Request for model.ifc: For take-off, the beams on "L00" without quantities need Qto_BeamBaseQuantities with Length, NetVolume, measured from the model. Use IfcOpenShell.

First a look at what the model holds.

```python
import ifcopenshell
import ifcopenshell.util.element
import ifcopenshell.util.unit

model = ifcopenshell.open("model.ifc")
print(model.schema)
for unit_type in ("LENGTHUNIT", "AREAUNIT", "VOLUMEUNIT"):
    print(unit_type, ifcopenshell.util.unit.calculate_unit_scale(model, unit_type))
storey = next(s for s in model.by_type("IfcBuildingStorey") if s.Name == "L00")
beams = [e for e in ifcopenshell.util.element.get_decomposition(storey) if e.is_a("IfcBeam")]
for e in sorted(beams, key=lambda e: e.id()):
    print(e.id(), e.is_a(), e.Name, list(ifcopenshell.util.element.get_psets(e, qtos_only=True)), sep=" | ")
```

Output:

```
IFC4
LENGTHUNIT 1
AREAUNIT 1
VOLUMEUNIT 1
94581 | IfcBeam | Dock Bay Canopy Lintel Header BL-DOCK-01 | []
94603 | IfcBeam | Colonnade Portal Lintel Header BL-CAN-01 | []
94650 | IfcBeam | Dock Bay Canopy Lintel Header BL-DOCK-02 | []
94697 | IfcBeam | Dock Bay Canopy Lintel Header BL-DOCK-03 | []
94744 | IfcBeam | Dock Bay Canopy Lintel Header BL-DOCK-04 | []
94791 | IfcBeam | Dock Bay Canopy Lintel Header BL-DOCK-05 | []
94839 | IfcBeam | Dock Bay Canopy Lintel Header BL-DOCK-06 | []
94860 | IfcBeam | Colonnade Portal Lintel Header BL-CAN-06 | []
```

```python
import ifcopenshell
import ifcopenshell.api.pset
import ifcopenshell.geom
import ifcopenshell.util.element
import ifcopenshell.util.shape
import ifcopenshell.util.unit

model = ifcopenshell.open("model.ifc")
unit_scale = ifcopenshell.util.unit.calculate_unit_scale(model)
volume_scale = ifcopenshell.util.unit.calculate_unit_scale(model, "VOLUMEUNIT")
settings = ifcopenshell.geom.settings()

storey = next(s for s in model.by_type("IfcBuildingStorey") if s.Name == "L00")
beams = [e for e in ifcopenshell.util.element.get_decomposition(storey) if e.is_a("IfcBeam")]

for e in sorted(beams, key=lambda e: e.id()):
    if ifcopenshell.util.element.get_psets(e, qtos_only=True, should_inherit=False):
        continue
    # Geometry comes back in metres, in the element's own axes.
    shape = ifcopenshell.geom.create_shape(settings, e)
    values = {
        "Length": ifcopenshell.util.shape.get_max_xyz(shape.geometry) / unit_scale,
        "NetVolume": ifcopenshell.util.shape.get_volume(shape.geometry) / volume_scale,
    }
    qto = ifcopenshell.api.pset.add_qto(model, product=e, name="Qto_BeamBaseQuantities")
    ifcopenshell.api.pset.edit_qto(model, qto=qto, properties=values)
    print(e.id(), {k: round(v, 3) for k, v in values.items()})

model.write("model_v2.ifc")
```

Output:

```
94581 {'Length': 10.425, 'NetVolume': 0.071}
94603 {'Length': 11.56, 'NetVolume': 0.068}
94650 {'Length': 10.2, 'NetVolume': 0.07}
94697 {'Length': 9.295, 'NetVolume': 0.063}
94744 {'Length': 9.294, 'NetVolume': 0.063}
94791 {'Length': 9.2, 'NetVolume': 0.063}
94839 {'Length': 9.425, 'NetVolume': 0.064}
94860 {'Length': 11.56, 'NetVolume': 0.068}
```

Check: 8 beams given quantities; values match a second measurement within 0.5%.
